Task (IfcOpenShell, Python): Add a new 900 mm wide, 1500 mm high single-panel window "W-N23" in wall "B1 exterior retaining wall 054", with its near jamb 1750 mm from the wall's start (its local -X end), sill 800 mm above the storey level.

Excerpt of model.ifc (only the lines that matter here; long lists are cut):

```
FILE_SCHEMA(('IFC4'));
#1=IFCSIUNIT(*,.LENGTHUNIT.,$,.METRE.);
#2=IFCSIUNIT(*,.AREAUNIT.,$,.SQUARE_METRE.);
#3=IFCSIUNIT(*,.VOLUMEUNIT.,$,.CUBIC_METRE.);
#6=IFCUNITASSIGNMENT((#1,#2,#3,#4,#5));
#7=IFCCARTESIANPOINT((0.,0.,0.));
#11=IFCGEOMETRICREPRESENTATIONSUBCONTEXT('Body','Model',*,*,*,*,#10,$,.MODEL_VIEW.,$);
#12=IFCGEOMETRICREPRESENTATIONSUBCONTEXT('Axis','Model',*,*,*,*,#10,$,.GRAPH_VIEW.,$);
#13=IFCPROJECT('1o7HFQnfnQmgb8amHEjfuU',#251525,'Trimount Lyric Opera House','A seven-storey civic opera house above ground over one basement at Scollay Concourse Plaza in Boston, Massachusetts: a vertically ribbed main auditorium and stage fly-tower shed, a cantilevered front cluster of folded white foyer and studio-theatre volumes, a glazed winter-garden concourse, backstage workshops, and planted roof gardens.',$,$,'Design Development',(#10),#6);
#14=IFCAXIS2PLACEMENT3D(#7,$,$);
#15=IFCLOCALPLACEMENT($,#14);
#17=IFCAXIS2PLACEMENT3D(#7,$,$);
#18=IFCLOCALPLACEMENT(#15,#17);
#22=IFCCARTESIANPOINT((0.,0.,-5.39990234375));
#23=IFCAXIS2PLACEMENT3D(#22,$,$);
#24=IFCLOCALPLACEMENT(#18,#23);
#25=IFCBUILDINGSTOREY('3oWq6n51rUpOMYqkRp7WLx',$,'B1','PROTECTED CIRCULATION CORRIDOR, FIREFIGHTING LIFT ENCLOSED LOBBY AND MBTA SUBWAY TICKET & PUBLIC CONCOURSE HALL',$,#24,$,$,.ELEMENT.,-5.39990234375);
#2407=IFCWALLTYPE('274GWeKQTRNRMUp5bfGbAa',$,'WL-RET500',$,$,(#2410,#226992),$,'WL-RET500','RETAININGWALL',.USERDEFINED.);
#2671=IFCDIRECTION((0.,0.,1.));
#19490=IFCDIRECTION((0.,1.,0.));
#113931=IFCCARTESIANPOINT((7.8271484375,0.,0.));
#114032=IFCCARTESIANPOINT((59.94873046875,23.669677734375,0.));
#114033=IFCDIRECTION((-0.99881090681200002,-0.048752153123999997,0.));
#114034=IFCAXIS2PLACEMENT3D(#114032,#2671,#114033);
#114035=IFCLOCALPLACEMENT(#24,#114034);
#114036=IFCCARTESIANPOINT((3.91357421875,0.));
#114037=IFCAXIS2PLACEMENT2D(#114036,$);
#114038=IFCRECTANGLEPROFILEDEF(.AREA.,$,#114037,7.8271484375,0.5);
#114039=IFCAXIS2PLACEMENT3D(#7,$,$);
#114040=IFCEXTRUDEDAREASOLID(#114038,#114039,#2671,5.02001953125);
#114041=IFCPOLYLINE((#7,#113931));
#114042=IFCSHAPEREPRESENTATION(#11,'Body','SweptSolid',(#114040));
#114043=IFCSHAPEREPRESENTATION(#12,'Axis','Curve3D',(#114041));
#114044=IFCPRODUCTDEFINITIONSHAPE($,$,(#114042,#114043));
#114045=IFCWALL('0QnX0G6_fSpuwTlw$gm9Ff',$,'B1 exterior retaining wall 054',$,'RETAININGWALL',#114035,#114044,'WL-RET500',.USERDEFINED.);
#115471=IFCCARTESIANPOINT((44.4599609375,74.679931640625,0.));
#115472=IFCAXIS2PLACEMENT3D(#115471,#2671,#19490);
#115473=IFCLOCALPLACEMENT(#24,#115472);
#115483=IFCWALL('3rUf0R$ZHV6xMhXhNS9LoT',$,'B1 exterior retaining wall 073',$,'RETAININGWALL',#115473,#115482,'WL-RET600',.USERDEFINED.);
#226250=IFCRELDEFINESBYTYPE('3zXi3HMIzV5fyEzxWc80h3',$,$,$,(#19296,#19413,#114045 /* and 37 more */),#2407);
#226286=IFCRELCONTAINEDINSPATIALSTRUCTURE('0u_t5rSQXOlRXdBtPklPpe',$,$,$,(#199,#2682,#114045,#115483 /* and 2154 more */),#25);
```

```python
import numpy as np
import ifcopenshell
import ifcopenshell.api.feature
import ifcopenshell.api.geometry
import ifcopenshell.api.root
import ifcopenshell.api.spatial
import ifcopenshell.geom
import ifcopenshell.util.element
import ifcopenshell.util.placement
import ifcopenshell.util.representation
import ifcopenshell.util.shape
import ifcopenshell.util.unit

model = ifcopenshell.open("model.ifc")
unit_scale = ifcopenshell.util.unit.calculate_unit_scale(model)
settings = ifcopenshell.geom.settings()


def volume(element):
    """Net volume in cubic metres, openings subtracted."""
    shape = ifcopenshell.geom.create_shape(settings, element)
    return ifcopenshell.util.shape.get_volume(shape.geometry)


wall = model.by_guid("0QnX0G6_fSpuwTlw$gm9Ff")
storey = ifcopenshell.util.element.get_container(wall, ifc_class="IfcBuildingStorey")
context = ifcopenshell.util.representation.get_context(model, "Model", "Body", "MODEL_VIEW")
before = volume(wall)

width, height, from_end, sill = 0.9, 1.5, 1.75, 0.8  # metres

# The wall runs along its own X axis, and the end named is its -X end.
wall_shape = ifcopenshell.geom.create_shape(settings, wall)
x, y, z = ifcopenshell.util.shape.get_vertices(wall_shape.geometry).T
start = x.min() + from_end
face, thickness = float(y.min()), float(y.max() - y.min())
wall_matrix = ifcopenshell.util.placement.get_local_placement(wall.ObjectPlacement)
level = ifcopenshell.util.placement.get_local_placement(storey.ObjectPlacement)[2, 3]


def in_wall(x, y):
    """Placement at x, y metres in the wall's axes, at sill height."""
    matrix = wall_matrix.copy()
    matrix[:, 3] = wall_matrix @ np.array([x / unit_scale, y / unit_scale, 0.0, 1.0])
    matrix[2, 3] = level + sill / unit_scale
    return matrix


# Opening: a box that overshoots both wall faces by 50 mm.
opening = ifcopenshell.api.root.create_entity(model, ifc_class="IfcOpeningElement", predefined_type="OPENING")
box = ifcopenshell.api.geometry.add_wall_representation(
    model, context=context, length=width, height=height, thickness=thickness + 0.1
)
ifcopenshell.api.geometry.assign_representation(model, product=opening, representation=box)
ifcopenshell.api.geometry.edit_object_placement(model, product=opening, matrix=in_wall(start, face - 0.05), is_si=False)
ifcopenshell.api.feature.add_feature(model, feature=opening, element=wall)

window = ifcopenshell.api.root.create_entity(model, ifc_class="IfcWindow", name="W-N23", predefined_type="WINDOW")
window.OverallWidth, window.OverallHeight = width / unit_scale, height / unit_scale
window.PartitioningType = "SINGLE_PANEL"
body = ifcopenshell.api.geometry.add_window_representation(
    model,
    context=context,
    overall_width=window.OverallWidth,
    overall_height=window.OverallHeight,
    partition_type="SINGLE_PANEL",
)
ifcopenshell.api.geometry.assign_representation(model, product=window, representation=body)
ifcopenshell.api.spatial.assign_container(model, products=[window], relating_structure=storey)
ifcopenshell.api.feature.add_filling(model, opening=opening, element=window)

# Centre the window in the wall's thickness.
ifcopenshell.api.geometry.edit_object_placement(model, product=window, matrix=in_wall(start, face), is_si=False)
window_shape = ifcopenshell.geom.create_shape(settings, window)
depth = ifcopenshell.util.shape.get_vertices(window_shape.geometry)[:, 1]
offset = face + thickness / 2 - (depth.min() + depth.max()) / 2
ifcopenshell.api.geometry.edit_object_placement(model, product=window, matrix=in_wall(start, offset), is_si=False)

after = volume(wall)

print(f"wall volume {before:.3f} -> {after:.3f} m3")

model.write("model-out.ifc")
```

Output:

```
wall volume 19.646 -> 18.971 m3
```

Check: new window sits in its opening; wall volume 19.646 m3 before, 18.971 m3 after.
